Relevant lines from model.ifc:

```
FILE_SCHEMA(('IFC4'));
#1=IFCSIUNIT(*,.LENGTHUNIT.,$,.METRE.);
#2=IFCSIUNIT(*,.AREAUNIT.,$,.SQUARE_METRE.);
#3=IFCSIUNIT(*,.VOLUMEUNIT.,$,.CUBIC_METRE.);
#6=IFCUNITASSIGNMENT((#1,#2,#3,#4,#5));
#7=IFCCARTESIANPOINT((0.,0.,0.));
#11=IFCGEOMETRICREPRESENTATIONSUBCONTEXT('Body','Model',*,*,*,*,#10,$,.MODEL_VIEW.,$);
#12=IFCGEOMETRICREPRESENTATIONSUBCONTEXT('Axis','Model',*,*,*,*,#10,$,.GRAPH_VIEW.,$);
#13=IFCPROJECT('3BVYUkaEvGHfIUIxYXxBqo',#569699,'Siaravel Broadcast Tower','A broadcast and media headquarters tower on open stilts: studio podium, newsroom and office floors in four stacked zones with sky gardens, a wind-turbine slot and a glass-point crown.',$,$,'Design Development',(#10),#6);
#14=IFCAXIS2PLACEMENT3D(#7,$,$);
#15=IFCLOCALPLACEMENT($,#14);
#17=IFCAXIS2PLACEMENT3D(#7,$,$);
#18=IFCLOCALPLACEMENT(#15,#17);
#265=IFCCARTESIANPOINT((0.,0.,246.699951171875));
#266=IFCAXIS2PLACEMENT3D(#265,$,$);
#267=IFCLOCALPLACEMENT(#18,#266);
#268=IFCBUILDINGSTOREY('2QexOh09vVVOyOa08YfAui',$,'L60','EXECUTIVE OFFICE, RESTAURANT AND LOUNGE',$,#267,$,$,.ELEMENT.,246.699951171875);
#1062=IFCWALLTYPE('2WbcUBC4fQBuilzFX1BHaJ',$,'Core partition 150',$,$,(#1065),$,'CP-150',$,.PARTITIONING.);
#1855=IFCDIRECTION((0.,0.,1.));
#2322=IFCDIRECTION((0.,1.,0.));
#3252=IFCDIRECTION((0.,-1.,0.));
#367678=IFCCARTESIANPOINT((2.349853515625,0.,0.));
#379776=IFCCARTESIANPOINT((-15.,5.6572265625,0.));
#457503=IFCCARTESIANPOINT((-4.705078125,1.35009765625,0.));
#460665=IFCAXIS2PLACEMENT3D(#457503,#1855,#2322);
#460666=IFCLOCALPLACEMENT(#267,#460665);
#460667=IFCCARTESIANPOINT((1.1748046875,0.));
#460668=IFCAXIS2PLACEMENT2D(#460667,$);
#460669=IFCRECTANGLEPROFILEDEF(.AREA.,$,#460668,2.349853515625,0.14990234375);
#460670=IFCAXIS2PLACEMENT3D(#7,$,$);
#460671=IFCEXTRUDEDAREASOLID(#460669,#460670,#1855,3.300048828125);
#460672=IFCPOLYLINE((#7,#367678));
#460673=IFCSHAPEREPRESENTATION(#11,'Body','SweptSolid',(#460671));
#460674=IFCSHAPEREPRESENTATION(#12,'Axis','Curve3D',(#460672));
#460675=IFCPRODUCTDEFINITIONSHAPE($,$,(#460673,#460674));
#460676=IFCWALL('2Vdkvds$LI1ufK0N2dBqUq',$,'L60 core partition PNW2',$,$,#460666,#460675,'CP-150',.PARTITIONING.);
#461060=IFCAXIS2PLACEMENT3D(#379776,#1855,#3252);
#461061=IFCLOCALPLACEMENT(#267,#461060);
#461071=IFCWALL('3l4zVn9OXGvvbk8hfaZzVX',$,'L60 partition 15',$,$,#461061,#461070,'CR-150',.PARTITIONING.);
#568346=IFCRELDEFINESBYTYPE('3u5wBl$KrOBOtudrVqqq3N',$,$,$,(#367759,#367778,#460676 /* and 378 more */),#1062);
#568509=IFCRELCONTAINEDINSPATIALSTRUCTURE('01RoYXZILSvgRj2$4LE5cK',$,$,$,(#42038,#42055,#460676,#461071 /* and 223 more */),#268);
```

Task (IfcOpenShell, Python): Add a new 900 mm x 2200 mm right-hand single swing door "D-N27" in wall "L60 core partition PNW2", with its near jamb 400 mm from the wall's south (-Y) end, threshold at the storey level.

```python
import numpy as np
import ifcopenshell
import ifcopenshell.api.feature
import ifcopenshell.api.geometry
import ifcopenshell.api.root
import ifcopenshell.api.spatial
import ifcopenshell.geom
import ifcopenshell.util.element
import ifcopenshell.util.placement
import ifcopenshell.util.representation
import ifcopenshell.util.shape
import ifcopenshell.util.unit

model = ifcopenshell.open("model.ifc")
unit_scale = ifcopenshell.util.unit.calculate_unit_scale(model)
settings = ifcopenshell.geom.settings()


def volume(element):
    """Net volume in cubic metres, openings subtracted."""
    shape = ifcopenshell.geom.create_shape(settings, element)
    return ifcopenshell.util.shape.get_volume(shape.geometry)


wall = model.by_guid("2Vdkvds$LI1ufK0N2dBqUq")
storey = ifcopenshell.util.element.get_container(wall, ifc_class="IfcBuildingStorey")
context = ifcopenshell.util.representation.get_context(model, "Model", "Body", "MODEL_VIEW")
before = volume(wall)

width, height, from_end, sill = 0.9, 2.2, 0.4, 0.0  # metres

# The wall runs along its own X axis, and the end named is its -X end.
wall_shape = ifcopenshell.geom.create_shape(settings, wall)
x, y, z = ifcopenshell.util.shape.get_vertices(wall_shape.geometry).T
start = x.min() + from_end
face, thickness = float(y.min()), float(y.max() - y.min())
wall_matrix = ifcopenshell.util.placement.get_local_placement(wall.ObjectPlacement)
level = ifcopenshell.util.placement.get_local_placement(storey.ObjectPlacement)[2, 3]


def in_wall(x, y):
    """Placement at x, y metres in the wall's axes, at sill height."""
    matrix = wall_matrix.copy()
    matrix[:, 3] = wall_matrix @ np.array([x / unit_scale, y / unit_scale, 0.0, 1.0])
    matrix[2, 3] = level + sill / unit_scale
    return matrix


# Opening: a box that overshoots both wall faces by 50 mm.
opening = ifcopenshell.api.root.create_entity(model, ifc_class="IfcOpeningElement", predefined_type="OPENING")
box = ifcopenshell.api.geometry.add_wall_representation(
    model, context=context, length=width, height=height, thickness=thickness + 0.1
)
ifcopenshell.api.geometry.assign_representation(model, product=opening, representation=box)
ifcopenshell.api.geometry.edit_object_placement(model, product=opening, matrix=in_wall(start, face - 0.05), is_si=False)
ifcopenshell.api.feature.add_feature(model, feature=opening, element=wall)

door = ifcopenshell.api.root.create_entity(model, ifc_class="IfcDoor", name="D-N27", predefined_type="DOOR")
door.OverallWidth, door.OverallHeight = width / unit_scale, height / unit_scale
door.OperationType = "SINGLE_SWING_RIGHT"
body = ifcopenshell.api.geometry.add_door_representation(
    model,
    context=context,
    overall_width=door.OverallWidth,
    overall_height=door.OverallHeight,
    operation_type="SINGLE_SWING_RIGHT",
    lining_properties={"LiningDepth": thickness / unit_scale, "ThresholdDepth": thickness / unit_scale},
)
ifcopenshell.api.geometry.assign_representation(model, product=door, representation=body)
ifcopenshell.api.spatial.assign_container(model, products=[door], relating_structure=storey)
ifcopenshell.api.feature.add_filling(model, opening=opening, element=door)

# The lining spans the wall, so the door starts at the wall face.
ifcopenshell.api.geometry.edit_object_placement(model, product=door, matrix=in_wall(start, face), is_si=False)

after = volume(wall)

print(f"wall volume {before:.3f} -> {after:.3f} m3")

model.write("model_edited.ifc")
```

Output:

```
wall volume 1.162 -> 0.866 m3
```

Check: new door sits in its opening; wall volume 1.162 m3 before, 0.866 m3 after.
